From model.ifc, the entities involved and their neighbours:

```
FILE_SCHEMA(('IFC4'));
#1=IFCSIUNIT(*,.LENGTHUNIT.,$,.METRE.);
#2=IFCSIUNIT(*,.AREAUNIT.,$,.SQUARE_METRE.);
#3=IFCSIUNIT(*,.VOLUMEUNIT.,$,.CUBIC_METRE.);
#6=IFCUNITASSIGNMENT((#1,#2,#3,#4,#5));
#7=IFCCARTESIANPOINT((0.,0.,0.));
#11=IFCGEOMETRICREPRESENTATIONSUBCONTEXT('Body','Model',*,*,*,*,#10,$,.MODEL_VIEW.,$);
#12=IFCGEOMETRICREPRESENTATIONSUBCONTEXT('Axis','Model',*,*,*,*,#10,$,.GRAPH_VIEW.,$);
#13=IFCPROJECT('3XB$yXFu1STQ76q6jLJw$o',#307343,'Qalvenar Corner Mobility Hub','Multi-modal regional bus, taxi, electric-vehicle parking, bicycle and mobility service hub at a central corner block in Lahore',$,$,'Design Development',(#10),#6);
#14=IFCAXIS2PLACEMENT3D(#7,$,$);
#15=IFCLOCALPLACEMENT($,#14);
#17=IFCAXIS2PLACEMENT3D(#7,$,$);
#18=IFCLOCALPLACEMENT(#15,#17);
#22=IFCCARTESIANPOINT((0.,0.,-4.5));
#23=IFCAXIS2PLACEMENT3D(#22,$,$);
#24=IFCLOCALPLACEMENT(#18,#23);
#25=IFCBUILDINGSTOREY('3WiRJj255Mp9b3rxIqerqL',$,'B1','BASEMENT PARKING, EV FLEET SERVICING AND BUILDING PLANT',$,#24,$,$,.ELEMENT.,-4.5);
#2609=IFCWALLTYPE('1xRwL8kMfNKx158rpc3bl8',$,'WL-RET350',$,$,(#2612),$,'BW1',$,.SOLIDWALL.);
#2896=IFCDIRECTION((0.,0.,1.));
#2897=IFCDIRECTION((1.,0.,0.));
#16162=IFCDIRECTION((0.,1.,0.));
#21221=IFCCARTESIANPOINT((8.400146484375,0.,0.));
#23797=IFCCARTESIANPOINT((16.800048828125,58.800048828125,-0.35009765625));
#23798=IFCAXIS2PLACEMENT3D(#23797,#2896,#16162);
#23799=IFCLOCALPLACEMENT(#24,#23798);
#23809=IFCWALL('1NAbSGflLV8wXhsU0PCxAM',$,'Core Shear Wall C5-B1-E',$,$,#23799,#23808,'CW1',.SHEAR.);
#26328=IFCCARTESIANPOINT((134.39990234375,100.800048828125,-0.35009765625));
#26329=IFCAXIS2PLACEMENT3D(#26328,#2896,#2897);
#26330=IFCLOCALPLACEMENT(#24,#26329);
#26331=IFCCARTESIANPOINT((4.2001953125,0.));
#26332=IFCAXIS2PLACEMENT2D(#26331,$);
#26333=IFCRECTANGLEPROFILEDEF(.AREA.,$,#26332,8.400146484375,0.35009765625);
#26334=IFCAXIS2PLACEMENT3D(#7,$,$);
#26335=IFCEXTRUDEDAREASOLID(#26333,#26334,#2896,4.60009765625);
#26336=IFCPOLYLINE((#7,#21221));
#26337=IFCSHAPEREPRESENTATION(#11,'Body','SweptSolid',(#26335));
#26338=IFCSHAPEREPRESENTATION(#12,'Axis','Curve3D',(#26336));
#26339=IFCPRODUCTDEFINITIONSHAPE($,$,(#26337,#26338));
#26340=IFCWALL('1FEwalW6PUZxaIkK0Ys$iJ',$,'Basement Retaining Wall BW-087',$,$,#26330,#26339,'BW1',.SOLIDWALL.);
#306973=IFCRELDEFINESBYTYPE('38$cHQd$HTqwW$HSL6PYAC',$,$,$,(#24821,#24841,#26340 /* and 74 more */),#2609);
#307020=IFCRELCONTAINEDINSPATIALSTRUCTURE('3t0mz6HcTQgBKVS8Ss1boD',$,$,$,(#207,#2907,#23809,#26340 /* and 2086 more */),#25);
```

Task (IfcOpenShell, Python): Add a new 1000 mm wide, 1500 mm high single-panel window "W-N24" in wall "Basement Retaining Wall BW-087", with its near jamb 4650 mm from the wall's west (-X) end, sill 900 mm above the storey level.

```python
import numpy as np
import ifcopenshell
import ifcopenshell.api.feature
import ifcopenshell.api.geometry
import ifcopenshell.api.root
import ifcopenshell.api.spatial
import ifcopenshell.geom
import ifcopenshell.util.element
import ifcopenshell.util.placement
import ifcopenshell.util.representation
import ifcopenshell.util.shape
import ifcopenshell.util.unit

model = ifcopenshell.open("model.ifc")
unit_scale = ifcopenshell.util.unit.calculate_unit_scale(model)
settings = ifcopenshell.geom.settings()


def volume(element):
    """Net volume in cubic metres, openings subtracted."""
    shape = ifcopenshell.geom.create_shape(settings, element)
    return ifcopenshell.util.shape.get_volume(shape.geometry)


wall = model.by_guid("1FEwalW6PUZxaIkK0Ys$iJ")
storey = ifcopenshell.util.element.get_container(wall, ifc_class="IfcBuildingStorey")
context = ifcopenshell.util.representation.get_context(model, "Model", "Body", "MODEL_VIEW")
before = volume(wall)

width, height, from_end, sill = 1, 1.5, 4.65, 0.9  # metres

# The wall runs along its own X axis, and the end named is its -X end.
wall_shape = ifcopenshell.geom.create_shape(settings, wall)
x, y, z = ifcopenshell.util.shape.get_vertices(wall_shape.geometry).T
start = x.min() + from_end
face, thickness = float(y.min()), float(y.max() - y.min())
wall_matrix = ifcopenshell.util.placement.get_local_placement(wall.ObjectPlacement)
level = ifcopenshell.util.placement.get_local_placement(storey.ObjectPlacement)[2, 3]


def in_wall(x, y):
    """Placement at x, y metres in the wall's axes, at sill height."""
    matrix = wall_matrix.copy()
    matrix[:, 3] = wall_matrix @ np.array([x / unit_scale, y / unit_scale, 0.0, 1.0])
    matrix[2, 3] = level + sill / unit_scale
    return matrix


# Opening: a box that overshoots both wall faces by 50 mm.
opening = ifcopenshell.api.root.create_entity(model, ifc_class="IfcOpeningElement", predefined_type="OPENING")
box = ifcopenshell.api.geometry.add_wall_representation(
    model, context=context, length=width, height=height, thickness=thickness + 0.1
)
ifcopenshell.api.geometry.assign_representation(model, product=opening, representation=box)
ifcopenshell.api.geometry.edit_object_placement(model, product=opening, matrix=in_wall(start, face - 0.05), is_si=False)
ifcopenshell.api.feature.add_feature(model, feature=opening, element=wall)

window = ifcopenshell.api.root.create_entity(model, ifc_class="IfcWindow", name="W-N24", predefined_type="WINDOW")
window.OverallWidth, window.OverallHeight = width / unit_scale, height / unit_scale
window.PartitioningType = "SINGLE_PANEL"
body = ifcopenshell.api.geometry.add_window_representation(
    model,
    context=context,
    overall_width=window.OverallWidth,
    overall_height=window.OverallHeight,
    partition_type="SINGLE_PANEL",
)
ifcopenshell.api.geometry.assign_representation(model, product=window, representation=body)
ifcopenshell.api.spatial.assign_container(model, products=[window], relating_structure=storey)
ifcopenshell.api.feature.add_filling(model, opening=opening, element=window)

# Centre the window in the wall's thickness.
ifcopenshell.api.geometry.edit_object_placement(model, product=window, matrix=in_wall(start, face), is_si=False)
window_shape = ifcopenshell.geom.create_shape(settings, window)
depth = ifcopenshell.util.shape.get_vertices(window_shape.geometry)[:, 1]
offset = face + thickness / 2 - (depth.min() + depth.max()) / 2
ifcopenshell.api.geometry.edit_object_placement(model, product=window, matrix=in_wall(start, offset), is_si=False)

after = volume(wall)

print(f"wall volume {before:.3f} -> {after:.3f} m3")

model.write("model_updated.ifc")
```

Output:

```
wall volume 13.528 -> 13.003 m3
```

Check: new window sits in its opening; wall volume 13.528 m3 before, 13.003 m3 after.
